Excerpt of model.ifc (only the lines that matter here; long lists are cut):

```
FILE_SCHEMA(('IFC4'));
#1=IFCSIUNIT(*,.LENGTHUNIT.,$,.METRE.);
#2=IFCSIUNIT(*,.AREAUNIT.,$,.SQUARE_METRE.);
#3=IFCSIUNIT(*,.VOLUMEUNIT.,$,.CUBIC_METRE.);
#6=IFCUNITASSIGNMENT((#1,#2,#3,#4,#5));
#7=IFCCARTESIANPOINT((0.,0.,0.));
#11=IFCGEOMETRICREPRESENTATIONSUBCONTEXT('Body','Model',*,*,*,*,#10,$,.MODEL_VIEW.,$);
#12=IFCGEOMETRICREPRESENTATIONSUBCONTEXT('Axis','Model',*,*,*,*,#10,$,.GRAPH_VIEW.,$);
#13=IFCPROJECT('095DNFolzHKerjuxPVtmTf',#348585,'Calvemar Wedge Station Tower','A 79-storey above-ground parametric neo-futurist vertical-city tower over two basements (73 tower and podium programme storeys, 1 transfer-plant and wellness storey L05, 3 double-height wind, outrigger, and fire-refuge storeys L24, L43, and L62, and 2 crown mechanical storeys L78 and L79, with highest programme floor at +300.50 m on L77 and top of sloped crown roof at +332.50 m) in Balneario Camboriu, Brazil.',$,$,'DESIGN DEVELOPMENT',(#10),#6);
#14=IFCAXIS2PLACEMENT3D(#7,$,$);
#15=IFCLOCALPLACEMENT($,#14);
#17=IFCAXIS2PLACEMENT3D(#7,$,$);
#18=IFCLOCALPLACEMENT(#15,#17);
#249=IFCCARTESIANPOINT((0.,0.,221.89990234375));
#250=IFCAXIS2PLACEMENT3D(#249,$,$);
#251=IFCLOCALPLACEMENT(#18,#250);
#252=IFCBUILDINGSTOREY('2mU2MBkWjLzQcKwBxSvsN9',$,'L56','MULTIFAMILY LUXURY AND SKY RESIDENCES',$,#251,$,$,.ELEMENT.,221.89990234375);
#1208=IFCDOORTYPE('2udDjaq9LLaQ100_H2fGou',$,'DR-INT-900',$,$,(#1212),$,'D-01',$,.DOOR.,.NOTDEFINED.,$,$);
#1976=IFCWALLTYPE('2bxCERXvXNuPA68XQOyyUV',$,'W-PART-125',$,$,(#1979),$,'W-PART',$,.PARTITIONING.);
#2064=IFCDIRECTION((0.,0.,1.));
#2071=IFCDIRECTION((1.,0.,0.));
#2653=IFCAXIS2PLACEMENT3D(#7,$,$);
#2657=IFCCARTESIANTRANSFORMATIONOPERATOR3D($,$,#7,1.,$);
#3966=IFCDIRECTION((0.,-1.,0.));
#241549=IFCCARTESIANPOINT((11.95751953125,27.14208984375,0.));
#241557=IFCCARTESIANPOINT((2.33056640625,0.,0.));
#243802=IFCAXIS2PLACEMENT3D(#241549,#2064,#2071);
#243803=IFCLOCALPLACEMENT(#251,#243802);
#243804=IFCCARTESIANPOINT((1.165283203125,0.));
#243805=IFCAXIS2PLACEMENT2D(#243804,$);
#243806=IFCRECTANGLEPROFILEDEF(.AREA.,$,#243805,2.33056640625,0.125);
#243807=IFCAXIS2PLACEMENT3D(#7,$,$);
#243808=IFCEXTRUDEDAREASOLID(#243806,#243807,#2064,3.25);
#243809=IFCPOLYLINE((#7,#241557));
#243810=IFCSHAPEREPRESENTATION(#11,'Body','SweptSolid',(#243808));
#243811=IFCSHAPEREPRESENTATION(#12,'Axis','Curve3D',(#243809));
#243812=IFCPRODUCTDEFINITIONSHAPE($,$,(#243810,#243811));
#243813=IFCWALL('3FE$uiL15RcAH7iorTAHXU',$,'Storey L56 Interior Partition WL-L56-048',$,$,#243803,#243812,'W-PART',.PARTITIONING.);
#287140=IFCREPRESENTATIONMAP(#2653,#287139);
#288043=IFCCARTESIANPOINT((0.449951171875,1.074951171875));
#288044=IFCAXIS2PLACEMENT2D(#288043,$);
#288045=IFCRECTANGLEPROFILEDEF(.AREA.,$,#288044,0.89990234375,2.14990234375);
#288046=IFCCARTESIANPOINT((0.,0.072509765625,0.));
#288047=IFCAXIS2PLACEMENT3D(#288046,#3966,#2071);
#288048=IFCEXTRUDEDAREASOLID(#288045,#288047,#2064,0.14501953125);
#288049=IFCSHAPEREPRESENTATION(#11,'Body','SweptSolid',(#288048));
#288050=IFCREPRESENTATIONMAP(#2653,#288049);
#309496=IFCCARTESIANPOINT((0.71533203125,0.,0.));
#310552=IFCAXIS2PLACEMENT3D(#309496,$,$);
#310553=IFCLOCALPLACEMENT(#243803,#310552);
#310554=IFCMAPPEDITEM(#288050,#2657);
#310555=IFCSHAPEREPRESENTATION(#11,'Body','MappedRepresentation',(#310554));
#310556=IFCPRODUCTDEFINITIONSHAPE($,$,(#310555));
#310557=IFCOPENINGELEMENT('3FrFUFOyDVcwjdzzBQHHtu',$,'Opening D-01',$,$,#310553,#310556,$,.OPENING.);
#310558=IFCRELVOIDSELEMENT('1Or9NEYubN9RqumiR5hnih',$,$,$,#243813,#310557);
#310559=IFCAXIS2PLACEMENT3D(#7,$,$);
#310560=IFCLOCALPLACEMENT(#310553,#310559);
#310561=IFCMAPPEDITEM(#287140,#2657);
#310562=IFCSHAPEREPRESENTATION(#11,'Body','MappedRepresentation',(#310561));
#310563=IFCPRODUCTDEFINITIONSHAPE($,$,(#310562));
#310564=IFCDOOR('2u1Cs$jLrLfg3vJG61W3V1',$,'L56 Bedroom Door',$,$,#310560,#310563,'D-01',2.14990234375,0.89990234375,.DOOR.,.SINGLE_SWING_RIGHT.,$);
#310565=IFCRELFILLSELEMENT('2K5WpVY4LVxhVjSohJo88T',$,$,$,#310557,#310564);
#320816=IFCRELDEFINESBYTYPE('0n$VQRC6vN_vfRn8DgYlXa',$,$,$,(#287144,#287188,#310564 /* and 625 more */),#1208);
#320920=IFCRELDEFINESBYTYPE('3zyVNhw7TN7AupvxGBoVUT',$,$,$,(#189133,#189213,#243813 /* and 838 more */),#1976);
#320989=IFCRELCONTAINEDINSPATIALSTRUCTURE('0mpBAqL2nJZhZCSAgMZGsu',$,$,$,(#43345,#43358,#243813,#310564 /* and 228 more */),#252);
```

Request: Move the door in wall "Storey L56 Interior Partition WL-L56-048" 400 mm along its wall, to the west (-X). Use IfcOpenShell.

```python
import ifcopenshell
import ifcopenshell.api.geometry
import ifcopenshell.util.placement
import ifcopenshell.util.unit

model = ifcopenshell.open("model.ifc")
unit_scale = ifcopenshell.util.unit.calculate_unit_scale(model)

door = model.by_guid("2u1Cs$jLrLfg3vJG61W3V1")
opening = door.FillsVoids[0].RelatingOpeningElement
wall = opening.VoidsElements[0].RelatingBuildingElement

wall_matrix = ifcopenshell.util.placement.get_local_placement(wall.ObjectPlacement)
shift = wall_matrix[:3, 0] * -0.4 / unit_scale
before = ifcopenshell.util.placement.get_local_placement(door.ObjectPlacement)[:3, 3].copy()

# The door is placed relative to its opening, so it follows when the opening moves.
matrix = ifcopenshell.util.placement.get_local_placement(opening.ObjectPlacement)
matrix[:3, 3] += shift
ifcopenshell.api.geometry.edit_object_placement(
    model, product=opening, matrix=matrix, is_si=False, should_transform_children=True
)

after = ifcopenshell.util.placement.get_local_placement(door.ObjectPlacement)[:3, 3]
print("door moved by", (after - before).round(3) + 0.0)

model.write("model_edited.ifc")
```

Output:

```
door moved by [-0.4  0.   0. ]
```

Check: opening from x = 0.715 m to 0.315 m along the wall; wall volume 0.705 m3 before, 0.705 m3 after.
